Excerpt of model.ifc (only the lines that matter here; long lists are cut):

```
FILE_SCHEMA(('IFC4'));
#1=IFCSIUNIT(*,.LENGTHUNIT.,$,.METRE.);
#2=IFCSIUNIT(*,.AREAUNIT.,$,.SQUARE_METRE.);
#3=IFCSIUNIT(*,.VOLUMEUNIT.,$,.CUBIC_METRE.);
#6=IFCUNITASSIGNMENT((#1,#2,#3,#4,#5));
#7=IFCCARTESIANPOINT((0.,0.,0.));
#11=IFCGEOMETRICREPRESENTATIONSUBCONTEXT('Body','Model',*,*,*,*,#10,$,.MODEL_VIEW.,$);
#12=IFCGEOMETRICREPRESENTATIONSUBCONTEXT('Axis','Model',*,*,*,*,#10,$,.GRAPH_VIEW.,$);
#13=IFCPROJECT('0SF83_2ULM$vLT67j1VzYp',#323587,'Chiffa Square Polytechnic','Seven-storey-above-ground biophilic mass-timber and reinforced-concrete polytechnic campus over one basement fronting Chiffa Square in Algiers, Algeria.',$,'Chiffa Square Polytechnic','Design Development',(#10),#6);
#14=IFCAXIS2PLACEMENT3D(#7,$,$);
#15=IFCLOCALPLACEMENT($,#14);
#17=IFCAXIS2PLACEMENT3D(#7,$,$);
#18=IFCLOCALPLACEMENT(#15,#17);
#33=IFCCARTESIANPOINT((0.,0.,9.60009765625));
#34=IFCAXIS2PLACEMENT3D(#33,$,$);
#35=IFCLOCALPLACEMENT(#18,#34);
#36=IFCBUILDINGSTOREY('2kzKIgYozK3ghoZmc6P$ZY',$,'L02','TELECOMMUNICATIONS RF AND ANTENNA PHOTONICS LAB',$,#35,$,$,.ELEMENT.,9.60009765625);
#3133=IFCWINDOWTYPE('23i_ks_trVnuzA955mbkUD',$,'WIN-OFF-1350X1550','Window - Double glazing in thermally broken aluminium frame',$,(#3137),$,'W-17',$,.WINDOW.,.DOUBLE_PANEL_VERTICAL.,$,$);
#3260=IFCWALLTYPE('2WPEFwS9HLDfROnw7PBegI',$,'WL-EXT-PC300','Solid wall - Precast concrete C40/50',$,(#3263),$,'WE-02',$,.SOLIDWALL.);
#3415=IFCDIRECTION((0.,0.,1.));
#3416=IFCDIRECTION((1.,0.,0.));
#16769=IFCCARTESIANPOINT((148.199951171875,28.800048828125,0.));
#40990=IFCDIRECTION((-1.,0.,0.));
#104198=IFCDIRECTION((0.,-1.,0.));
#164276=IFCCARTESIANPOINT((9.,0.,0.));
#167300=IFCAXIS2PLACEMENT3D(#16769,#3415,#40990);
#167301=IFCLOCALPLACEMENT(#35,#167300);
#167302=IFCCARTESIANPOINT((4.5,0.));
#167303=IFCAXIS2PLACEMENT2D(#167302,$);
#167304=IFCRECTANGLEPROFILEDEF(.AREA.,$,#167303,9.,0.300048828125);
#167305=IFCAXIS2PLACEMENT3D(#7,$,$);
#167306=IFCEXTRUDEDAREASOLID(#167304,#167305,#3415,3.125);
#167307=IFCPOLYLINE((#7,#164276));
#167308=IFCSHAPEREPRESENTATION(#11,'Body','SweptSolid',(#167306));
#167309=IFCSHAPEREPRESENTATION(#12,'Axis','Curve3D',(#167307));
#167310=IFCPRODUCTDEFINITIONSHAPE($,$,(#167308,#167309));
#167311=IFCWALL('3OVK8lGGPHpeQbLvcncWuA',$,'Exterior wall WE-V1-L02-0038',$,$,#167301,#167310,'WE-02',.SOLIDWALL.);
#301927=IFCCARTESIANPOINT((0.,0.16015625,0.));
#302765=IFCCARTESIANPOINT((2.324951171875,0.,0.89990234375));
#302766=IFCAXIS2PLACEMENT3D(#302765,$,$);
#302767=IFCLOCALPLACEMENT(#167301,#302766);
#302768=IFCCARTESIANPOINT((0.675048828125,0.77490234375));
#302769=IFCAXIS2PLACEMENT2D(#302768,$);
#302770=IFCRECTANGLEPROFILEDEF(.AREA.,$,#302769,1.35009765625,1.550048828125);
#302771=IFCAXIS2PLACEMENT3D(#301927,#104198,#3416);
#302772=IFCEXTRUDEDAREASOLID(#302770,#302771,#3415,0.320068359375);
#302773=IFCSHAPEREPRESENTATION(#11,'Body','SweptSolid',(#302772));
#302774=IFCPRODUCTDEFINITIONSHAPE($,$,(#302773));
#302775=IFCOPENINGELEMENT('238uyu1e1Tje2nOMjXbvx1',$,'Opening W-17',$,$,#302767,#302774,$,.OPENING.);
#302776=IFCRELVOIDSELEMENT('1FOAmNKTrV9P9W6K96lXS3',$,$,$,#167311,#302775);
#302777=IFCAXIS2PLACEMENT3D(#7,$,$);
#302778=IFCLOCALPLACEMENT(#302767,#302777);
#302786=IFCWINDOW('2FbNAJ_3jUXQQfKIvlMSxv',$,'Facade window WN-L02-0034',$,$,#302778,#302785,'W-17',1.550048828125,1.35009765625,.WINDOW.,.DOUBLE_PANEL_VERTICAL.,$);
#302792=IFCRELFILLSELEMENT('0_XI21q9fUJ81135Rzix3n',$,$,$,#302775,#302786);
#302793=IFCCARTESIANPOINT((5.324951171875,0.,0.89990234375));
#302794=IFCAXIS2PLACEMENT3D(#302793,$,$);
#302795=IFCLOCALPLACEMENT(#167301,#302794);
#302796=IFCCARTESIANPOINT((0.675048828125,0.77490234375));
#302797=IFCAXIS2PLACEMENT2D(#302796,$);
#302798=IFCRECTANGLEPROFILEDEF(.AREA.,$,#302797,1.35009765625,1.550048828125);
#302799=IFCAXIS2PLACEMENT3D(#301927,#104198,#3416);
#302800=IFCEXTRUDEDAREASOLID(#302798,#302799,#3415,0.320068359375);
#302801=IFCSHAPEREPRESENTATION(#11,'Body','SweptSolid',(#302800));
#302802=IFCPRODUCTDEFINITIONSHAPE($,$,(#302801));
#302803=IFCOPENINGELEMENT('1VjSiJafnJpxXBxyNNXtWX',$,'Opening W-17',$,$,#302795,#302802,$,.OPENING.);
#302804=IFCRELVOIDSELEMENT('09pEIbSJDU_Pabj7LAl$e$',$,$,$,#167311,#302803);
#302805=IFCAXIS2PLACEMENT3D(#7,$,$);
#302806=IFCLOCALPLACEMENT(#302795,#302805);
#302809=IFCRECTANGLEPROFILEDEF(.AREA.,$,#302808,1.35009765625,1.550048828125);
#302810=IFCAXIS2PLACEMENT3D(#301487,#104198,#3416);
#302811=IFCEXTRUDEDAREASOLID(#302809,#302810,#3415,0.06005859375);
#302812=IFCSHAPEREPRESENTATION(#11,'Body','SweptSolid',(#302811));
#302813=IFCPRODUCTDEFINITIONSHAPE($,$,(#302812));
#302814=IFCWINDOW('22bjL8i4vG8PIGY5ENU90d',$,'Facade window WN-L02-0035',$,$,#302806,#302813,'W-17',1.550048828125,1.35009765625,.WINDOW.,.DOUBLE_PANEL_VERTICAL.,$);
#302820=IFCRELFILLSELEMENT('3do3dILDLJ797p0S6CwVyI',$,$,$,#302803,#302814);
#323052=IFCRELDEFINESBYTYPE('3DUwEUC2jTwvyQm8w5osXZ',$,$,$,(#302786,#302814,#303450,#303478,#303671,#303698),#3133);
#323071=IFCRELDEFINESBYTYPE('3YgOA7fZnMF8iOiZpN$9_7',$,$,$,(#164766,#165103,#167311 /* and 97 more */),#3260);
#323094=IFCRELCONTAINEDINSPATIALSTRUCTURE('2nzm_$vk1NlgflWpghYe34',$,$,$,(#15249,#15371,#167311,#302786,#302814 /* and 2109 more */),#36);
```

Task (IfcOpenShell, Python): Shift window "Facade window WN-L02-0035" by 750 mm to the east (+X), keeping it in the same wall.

```python
import ifcopenshell
import ifcopenshell.api.geometry
import ifcopenshell.util.placement

model = ifcopenshell.open("model.ifc")

window = model.by_guid("22bjL8i4vG8PIGY5ENU90d")
opening = window.FillsVoids[0].RelatingOpeningElement
wall = opening.VoidsElements[0].RelatingBuildingElement

wall_matrix = ifcopenshell.util.placement.get_local_placement(wall.ObjectPlacement)
shift = wall_matrix[:3, 0] * -0.75
before = ifcopenshell.util.placement.get_local_placement(window.ObjectPlacement)[:3, 3].copy()

# The window is placed relative to its opening, so it follows when the opening moves.
matrix = ifcopenshell.util.placement.get_local_placement(opening.ObjectPlacement)
matrix[:3, 3] += shift
ifcopenshell.api.geometry.edit_object_placement(
    model, product=opening, matrix=matrix, is_si=False, should_transform_children=True
)

after = ifcopenshell.util.placement.get_local_placement(window.ObjectPlacement)[:3, 3]
print("window moved by", (after - before).round(3) + 0.0)

model.write("model_rev.ifc")
```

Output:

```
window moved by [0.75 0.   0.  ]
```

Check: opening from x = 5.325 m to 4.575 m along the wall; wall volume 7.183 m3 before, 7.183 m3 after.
